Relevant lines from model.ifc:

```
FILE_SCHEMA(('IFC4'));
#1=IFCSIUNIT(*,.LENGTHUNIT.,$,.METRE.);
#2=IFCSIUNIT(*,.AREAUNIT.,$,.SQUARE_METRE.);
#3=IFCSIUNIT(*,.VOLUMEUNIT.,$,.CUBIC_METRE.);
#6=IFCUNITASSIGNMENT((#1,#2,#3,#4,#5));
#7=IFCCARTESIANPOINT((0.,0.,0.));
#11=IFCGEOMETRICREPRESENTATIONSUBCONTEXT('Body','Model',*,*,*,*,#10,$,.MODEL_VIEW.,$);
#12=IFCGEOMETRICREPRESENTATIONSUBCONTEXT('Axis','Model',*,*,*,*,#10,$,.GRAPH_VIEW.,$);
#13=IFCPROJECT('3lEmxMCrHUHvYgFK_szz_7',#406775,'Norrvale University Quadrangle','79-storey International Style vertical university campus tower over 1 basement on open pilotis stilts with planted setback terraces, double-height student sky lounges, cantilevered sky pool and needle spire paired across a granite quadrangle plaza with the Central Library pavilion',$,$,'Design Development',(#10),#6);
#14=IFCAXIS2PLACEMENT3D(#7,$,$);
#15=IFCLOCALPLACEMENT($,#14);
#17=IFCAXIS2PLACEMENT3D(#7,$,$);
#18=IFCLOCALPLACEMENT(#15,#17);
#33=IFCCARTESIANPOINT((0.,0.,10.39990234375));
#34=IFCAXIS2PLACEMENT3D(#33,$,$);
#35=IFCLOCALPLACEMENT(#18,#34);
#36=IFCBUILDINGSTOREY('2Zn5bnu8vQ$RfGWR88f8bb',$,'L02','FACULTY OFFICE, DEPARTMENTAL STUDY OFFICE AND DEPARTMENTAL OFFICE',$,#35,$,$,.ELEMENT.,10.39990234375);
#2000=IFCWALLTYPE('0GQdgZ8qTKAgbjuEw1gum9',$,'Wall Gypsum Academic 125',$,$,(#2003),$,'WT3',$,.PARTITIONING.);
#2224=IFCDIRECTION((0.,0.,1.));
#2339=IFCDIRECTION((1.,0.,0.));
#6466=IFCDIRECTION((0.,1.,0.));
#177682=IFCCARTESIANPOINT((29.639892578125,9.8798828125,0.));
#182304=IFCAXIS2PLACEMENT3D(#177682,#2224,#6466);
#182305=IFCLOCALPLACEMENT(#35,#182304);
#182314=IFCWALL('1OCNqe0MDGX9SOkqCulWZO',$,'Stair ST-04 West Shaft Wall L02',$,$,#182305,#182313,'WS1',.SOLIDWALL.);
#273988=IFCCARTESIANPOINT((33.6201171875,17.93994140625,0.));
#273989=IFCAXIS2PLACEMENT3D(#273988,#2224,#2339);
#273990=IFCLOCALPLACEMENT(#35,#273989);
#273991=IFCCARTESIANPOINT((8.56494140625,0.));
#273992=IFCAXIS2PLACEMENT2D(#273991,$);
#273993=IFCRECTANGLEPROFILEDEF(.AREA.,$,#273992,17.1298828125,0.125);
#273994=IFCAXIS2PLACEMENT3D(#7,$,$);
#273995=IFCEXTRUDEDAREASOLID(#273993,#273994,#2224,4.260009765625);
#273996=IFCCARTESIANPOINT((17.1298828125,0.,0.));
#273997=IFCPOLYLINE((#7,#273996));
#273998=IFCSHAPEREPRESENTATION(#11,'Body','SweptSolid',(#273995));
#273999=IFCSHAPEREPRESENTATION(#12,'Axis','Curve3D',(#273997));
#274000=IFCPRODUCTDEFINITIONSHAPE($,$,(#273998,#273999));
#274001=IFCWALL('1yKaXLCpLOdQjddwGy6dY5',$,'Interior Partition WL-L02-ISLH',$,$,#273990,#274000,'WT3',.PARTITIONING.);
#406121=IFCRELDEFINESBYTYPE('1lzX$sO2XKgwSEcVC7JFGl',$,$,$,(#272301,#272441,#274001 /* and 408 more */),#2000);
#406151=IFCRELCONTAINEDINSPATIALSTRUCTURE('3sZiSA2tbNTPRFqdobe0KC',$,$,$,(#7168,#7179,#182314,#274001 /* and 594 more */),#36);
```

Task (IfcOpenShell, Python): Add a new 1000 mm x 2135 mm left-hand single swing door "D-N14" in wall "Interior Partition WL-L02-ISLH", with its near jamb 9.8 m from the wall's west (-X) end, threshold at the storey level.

```python
import numpy as np
import ifcopenshell
import ifcopenshell.api.feature
import ifcopenshell.api.geometry
import ifcopenshell.api.root
import ifcopenshell.api.spatial
import ifcopenshell.geom
import ifcopenshell.util.element
import ifcopenshell.util.placement
import ifcopenshell.util.representation
import ifcopenshell.util.shape
import ifcopenshell.util.unit

model = ifcopenshell.open("model.ifc")
unit_scale = ifcopenshell.util.unit.calculate_unit_scale(model)
settings = ifcopenshell.geom.settings()


def volume(element):
    """Net volume in cubic metres, openings subtracted."""
    shape = ifcopenshell.geom.create_shape(settings, element)
    return ifcopenshell.util.shape.get_volume(shape.geometry)


wall = model.by_guid("1yKaXLCpLOdQjddwGy6dY5")
storey = ifcopenshell.util.element.get_container(wall, ifc_class="IfcBuildingStorey")
context = ifcopenshell.util.representation.get_context(model, "Model", "Body", "MODEL_VIEW")
before = volume(wall)

width, height, from_end, sill = 1, 2.135, 9.8, 0.0  # metres

# The wall runs along its own X axis, and the end named is its -X end.
wall_shape = ifcopenshell.geom.create_shape(settings, wall)
x, y, z = ifcopenshell.util.shape.get_vertices(wall_shape.geometry).T
start = x.min() + from_end
face, thickness = float(y.min()), float(y.max() - y.min())
wall_matrix = ifcopenshell.util.placement.get_local_placement(wall.ObjectPlacement)
level = ifcopenshell.util.placement.get_local_placement(storey.ObjectPlacement)[2, 3]


def in_wall(x, y):
    """Placement at x, y metres in the wall's axes, at sill height."""
    matrix = wall_matrix.copy()
    matrix[:, 3] = wall_matrix @ np.array([x / unit_scale, y / unit_scale, 0.0, 1.0])
    matrix[2, 3] = level + sill / unit_scale
    return matrix


# Opening: a box that overshoots both wall faces by 50 mm.
opening = ifcopenshell.api.root.create_entity(model, ifc_class="IfcOpeningElement", predefined_type="OPENING")
box = ifcopenshell.api.geometry.add_wall_representation(
    model, context=context, length=width, height=height, thickness=thickness + 0.1
)
ifcopenshell.api.geometry.assign_representation(model, product=opening, representation=box)
ifcopenshell.api.geometry.edit_object_placement(model, product=opening, matrix=in_wall(start, face - 0.05), is_si=False)
ifcopenshell.api.feature.add_feature(model, feature=opening, element=wall)

door = ifcopenshell.api.root.create_entity(model, ifc_class="IfcDoor", name="D-N14", predefined_type="DOOR")
door.OverallWidth, door.OverallHeight = width / unit_scale, height / unit_scale
door.OperationType = "SINGLE_SWING_LEFT"
body = ifcopenshell.api.geometry.add_door_representation(
    model,
    context=context,
    overall_width=door.OverallWidth,
    overall_height=door.OverallHeight,
    operation_type="SINGLE_SWING_LEFT",
    lining_properties={"LiningDepth": thickness / unit_scale, "ThresholdDepth": thickness / unit_scale},
)
ifcopenshell.api.geometry.assign_representation(model, product=door, representation=body)
ifcopenshell.api.spatial.assign_container(model, products=[door], relating_structure=storey)
ifcopenshell.api.feature.add_filling(model, opening=opening, element=door)

# The lining spans the wall, so the door starts at the wall face.
ifcopenshell.api.geometry.edit_object_placement(model, product=door, matrix=in_wall(start, face), is_si=False)

after = volume(wall)

print(f"wall volume {before:.3f} -> {after:.3f} m3")

model.write("model-out.ifc")
```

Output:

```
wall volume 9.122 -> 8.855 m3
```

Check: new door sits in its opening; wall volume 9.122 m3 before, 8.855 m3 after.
